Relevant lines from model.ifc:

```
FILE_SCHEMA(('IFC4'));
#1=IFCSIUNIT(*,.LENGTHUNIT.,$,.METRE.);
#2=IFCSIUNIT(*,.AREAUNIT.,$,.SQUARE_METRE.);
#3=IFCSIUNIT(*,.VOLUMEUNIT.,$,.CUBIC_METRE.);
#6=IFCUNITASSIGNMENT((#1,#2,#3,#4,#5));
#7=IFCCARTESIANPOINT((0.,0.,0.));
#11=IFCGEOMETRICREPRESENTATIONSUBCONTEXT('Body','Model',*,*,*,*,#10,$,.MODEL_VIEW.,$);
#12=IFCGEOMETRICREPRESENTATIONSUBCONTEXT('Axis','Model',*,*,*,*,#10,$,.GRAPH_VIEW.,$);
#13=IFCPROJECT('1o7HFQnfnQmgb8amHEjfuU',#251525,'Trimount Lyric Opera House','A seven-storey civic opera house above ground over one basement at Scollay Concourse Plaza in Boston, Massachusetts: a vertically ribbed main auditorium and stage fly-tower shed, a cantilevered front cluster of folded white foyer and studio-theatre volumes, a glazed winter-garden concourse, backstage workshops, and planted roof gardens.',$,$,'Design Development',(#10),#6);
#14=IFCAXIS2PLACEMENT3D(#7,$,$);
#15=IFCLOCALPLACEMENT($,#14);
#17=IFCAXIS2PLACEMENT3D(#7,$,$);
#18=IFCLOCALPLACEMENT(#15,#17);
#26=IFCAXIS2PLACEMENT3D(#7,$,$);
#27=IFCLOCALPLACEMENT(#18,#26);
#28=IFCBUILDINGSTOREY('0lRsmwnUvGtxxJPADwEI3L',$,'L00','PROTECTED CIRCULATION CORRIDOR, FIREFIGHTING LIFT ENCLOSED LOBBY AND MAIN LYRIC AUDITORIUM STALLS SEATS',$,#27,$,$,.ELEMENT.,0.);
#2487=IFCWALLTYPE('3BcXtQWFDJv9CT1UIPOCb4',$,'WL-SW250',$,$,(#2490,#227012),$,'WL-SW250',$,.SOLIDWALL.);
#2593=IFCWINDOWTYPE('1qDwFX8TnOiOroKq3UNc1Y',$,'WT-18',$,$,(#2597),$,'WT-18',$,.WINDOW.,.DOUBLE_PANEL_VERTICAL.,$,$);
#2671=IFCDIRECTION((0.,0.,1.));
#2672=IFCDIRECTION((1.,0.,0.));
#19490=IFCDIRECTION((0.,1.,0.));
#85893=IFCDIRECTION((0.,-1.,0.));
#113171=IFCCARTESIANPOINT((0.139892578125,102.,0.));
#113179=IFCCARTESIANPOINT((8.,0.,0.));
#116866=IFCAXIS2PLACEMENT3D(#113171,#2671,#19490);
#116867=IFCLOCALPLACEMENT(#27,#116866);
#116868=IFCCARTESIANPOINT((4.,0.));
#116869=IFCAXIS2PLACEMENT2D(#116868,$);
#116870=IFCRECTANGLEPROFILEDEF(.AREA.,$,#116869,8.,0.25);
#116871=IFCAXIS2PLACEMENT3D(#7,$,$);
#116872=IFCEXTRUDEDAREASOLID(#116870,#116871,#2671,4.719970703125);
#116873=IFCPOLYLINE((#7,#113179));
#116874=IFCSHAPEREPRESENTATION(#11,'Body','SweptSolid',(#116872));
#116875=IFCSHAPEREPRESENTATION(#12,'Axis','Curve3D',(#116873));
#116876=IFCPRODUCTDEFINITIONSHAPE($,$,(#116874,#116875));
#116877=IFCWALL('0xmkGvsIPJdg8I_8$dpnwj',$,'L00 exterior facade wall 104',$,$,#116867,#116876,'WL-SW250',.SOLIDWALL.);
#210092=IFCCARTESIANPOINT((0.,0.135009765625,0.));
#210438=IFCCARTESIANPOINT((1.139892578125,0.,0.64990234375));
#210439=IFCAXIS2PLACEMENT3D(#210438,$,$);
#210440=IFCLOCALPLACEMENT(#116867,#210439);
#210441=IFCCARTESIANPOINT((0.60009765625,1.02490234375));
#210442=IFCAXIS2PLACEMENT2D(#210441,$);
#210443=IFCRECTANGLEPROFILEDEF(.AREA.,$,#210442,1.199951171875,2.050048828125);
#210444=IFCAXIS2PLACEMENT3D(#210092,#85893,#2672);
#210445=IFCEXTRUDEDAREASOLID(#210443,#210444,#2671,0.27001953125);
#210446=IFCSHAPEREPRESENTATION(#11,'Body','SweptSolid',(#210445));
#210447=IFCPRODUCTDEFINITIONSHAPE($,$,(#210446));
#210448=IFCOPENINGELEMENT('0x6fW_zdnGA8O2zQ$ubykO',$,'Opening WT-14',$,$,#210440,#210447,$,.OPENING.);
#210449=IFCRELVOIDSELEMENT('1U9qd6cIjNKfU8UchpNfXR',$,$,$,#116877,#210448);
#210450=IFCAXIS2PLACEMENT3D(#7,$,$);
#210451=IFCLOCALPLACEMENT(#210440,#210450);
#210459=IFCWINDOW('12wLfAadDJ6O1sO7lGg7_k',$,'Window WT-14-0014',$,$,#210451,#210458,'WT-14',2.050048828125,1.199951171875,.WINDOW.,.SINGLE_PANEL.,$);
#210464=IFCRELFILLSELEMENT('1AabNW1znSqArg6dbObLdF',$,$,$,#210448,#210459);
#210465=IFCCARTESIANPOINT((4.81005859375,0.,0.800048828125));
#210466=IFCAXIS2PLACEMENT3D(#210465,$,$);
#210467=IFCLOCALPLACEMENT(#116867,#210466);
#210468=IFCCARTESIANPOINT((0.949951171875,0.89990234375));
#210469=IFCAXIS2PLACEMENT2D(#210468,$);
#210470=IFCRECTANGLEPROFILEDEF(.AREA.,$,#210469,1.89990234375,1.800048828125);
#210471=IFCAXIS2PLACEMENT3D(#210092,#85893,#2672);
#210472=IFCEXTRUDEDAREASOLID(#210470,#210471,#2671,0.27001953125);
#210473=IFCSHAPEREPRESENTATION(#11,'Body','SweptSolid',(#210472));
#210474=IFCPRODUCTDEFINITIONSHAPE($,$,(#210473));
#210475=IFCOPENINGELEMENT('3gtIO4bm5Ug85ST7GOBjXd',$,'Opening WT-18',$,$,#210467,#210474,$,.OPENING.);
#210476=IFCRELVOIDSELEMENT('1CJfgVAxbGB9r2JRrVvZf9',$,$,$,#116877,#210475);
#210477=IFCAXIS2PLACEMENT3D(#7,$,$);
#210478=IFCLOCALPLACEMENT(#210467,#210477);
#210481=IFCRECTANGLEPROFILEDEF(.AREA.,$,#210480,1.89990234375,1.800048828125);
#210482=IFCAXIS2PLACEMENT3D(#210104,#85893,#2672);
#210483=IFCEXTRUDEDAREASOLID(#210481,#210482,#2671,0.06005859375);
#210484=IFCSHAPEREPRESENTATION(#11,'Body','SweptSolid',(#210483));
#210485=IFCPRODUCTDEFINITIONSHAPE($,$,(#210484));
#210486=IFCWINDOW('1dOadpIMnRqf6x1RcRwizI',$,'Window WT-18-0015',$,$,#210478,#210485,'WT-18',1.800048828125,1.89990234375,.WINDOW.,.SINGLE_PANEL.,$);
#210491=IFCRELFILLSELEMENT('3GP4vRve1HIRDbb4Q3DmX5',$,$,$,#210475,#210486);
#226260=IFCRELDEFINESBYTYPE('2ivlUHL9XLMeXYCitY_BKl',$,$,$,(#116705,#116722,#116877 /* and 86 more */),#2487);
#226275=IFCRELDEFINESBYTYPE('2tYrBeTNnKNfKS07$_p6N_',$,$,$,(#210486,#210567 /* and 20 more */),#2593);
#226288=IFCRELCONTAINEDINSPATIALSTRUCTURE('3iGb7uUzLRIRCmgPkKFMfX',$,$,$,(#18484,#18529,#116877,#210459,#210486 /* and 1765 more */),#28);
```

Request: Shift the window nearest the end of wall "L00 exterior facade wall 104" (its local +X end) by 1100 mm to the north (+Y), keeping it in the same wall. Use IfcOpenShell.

```python
import ifcopenshell
import ifcopenshell.api.geometry
import ifcopenshell.util.placement
import ifcopenshell.util.unit

model = ifcopenshell.open("model.ifc")
unit_scale = ifcopenshell.util.unit.calculate_unit_scale(model)

window = model.by_guid("1dOadpIMnRqf6x1RcRwizI")
opening = window.FillsVoids[0].RelatingOpeningElement
wall = opening.VoidsElements[0].RelatingBuildingElement

wall_matrix = ifcopenshell.util.placement.get_local_placement(wall.ObjectPlacement)
shift = wall_matrix[:3, 0] * 1.1 / unit_scale
before = ifcopenshell.util.placement.get_local_placement(window.ObjectPlacement)[:3, 3].copy()

# The window is placed relative to its opening, so it follows when the opening moves.
matrix = ifcopenshell.util.placement.get_local_placement(opening.ObjectPlacement)
matrix[:3, 3] += shift
ifcopenshell.api.geometry.edit_object_placement(
    model, product=opening, matrix=matrix, is_si=False, should_transform_children=True
)

after = ifcopenshell.util.placement.get_local_placement(window.ObjectPlacement)[:3, 3]
print("window moved by", (after - before).round(3) + 0.0)

model.write("model_edited.ifc")
```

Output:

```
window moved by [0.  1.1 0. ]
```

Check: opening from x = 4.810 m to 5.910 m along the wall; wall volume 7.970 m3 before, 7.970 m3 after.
